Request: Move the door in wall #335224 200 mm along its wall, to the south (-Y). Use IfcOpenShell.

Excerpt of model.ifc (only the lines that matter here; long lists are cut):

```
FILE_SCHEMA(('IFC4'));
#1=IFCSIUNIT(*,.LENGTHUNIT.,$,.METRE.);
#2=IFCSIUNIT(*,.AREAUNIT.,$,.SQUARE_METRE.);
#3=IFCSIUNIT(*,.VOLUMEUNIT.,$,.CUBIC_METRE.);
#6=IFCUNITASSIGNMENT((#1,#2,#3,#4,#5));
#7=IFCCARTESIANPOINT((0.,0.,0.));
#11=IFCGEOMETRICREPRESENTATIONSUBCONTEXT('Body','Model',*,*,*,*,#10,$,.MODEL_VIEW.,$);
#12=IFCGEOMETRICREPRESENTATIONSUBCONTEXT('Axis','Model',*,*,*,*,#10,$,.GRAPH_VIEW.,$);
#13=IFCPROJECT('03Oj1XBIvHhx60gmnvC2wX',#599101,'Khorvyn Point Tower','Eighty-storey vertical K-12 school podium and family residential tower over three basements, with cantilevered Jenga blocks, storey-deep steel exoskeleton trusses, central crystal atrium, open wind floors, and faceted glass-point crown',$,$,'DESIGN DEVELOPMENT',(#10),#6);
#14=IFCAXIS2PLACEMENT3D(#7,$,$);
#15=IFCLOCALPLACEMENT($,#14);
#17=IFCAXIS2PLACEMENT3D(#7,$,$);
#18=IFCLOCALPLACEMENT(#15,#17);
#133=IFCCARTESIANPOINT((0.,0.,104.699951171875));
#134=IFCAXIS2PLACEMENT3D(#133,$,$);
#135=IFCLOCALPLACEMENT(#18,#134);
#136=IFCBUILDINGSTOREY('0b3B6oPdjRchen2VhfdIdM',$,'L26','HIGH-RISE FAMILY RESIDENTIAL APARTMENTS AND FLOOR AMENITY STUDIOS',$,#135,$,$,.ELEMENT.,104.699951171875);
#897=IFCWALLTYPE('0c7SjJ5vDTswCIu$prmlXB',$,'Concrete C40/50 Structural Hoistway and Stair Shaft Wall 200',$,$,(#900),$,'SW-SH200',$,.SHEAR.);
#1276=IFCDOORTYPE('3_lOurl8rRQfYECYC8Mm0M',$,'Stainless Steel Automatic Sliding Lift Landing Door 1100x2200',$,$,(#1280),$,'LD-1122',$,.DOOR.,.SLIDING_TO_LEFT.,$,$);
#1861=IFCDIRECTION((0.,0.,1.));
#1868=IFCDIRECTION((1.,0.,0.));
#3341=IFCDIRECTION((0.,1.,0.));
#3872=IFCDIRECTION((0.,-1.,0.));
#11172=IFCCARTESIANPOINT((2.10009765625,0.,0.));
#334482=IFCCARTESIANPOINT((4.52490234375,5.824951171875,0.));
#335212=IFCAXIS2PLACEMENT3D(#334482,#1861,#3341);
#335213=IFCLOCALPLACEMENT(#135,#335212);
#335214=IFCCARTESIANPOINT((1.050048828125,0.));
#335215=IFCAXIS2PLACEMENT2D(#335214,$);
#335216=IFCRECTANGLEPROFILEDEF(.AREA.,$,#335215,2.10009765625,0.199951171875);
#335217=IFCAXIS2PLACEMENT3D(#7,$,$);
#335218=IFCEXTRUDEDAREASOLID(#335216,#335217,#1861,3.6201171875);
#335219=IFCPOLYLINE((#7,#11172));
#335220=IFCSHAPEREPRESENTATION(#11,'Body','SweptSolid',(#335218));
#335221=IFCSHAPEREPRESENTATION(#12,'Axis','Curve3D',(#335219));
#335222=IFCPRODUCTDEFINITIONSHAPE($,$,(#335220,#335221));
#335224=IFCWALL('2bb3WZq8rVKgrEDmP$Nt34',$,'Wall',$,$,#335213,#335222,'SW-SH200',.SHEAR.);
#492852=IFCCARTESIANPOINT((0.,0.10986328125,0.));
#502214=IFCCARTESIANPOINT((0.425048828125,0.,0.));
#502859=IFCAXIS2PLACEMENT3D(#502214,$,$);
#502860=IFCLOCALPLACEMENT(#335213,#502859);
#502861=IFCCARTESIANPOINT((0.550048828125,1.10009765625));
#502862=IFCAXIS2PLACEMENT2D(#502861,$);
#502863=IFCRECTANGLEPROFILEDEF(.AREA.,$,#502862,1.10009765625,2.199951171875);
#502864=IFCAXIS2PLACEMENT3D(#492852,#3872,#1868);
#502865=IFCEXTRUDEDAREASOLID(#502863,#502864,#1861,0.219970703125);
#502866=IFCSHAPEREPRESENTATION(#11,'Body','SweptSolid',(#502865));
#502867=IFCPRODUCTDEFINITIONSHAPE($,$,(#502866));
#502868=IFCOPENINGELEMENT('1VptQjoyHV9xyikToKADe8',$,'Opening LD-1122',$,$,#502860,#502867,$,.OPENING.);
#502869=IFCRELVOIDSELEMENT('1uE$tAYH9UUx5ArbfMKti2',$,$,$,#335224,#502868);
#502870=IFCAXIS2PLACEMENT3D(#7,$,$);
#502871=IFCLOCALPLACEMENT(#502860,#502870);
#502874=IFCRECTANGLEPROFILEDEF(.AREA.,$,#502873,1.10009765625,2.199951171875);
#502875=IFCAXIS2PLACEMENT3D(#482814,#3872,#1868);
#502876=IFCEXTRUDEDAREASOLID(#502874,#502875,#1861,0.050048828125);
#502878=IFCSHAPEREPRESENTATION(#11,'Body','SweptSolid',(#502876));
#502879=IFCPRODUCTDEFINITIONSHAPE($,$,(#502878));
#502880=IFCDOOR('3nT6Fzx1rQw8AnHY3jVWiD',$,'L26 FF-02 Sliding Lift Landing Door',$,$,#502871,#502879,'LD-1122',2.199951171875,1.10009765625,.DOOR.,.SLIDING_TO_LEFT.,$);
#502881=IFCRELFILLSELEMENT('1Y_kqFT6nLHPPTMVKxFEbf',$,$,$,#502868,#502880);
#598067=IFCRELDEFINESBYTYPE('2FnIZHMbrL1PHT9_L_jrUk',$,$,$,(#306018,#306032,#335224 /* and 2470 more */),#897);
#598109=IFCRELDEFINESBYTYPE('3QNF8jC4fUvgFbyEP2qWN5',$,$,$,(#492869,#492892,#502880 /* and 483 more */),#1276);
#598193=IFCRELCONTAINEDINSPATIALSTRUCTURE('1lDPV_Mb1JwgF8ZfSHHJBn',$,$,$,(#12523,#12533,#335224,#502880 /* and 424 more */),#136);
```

```python
import ifcopenshell
import ifcopenshell.api.geometry
import ifcopenshell.util.placement
import ifcopenshell.util.unit

model = ifcopenshell.open("model.ifc")
unit_scale = ifcopenshell.util.unit.calculate_unit_scale(model)

door = model.by_guid("3nT6Fzx1rQw8AnHY3jVWiD")
opening = door.FillsVoids[0].RelatingOpeningElement
wall = opening.VoidsElements[0].RelatingBuildingElement

wall_matrix = ifcopenshell.util.placement.get_local_placement(wall.ObjectPlacement)
shift = wall_matrix[:3, 0] * -0.2 / unit_scale
before = ifcopenshell.util.placement.get_local_placement(door.ObjectPlacement)[:3, 3].copy()

# The door is placed relative to its opening, so it follows when the opening moves.
matrix = ifcopenshell.util.placement.get_local_placement(opening.ObjectPlacement)
matrix[:3, 3] += shift
ifcopenshell.api.geometry.edit_object_placement(
    model, product=opening, matrix=matrix, is_si=False, should_transform_children=True
)

after = ifcopenshell.util.placement.get_local_placement(door.ObjectPlacement)[:3, 3]
print("door moved by", (after - before).round(3) + 0.0)

model.write("model-out.ifc")
```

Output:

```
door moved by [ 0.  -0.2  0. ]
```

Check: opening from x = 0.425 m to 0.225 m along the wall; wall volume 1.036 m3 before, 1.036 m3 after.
